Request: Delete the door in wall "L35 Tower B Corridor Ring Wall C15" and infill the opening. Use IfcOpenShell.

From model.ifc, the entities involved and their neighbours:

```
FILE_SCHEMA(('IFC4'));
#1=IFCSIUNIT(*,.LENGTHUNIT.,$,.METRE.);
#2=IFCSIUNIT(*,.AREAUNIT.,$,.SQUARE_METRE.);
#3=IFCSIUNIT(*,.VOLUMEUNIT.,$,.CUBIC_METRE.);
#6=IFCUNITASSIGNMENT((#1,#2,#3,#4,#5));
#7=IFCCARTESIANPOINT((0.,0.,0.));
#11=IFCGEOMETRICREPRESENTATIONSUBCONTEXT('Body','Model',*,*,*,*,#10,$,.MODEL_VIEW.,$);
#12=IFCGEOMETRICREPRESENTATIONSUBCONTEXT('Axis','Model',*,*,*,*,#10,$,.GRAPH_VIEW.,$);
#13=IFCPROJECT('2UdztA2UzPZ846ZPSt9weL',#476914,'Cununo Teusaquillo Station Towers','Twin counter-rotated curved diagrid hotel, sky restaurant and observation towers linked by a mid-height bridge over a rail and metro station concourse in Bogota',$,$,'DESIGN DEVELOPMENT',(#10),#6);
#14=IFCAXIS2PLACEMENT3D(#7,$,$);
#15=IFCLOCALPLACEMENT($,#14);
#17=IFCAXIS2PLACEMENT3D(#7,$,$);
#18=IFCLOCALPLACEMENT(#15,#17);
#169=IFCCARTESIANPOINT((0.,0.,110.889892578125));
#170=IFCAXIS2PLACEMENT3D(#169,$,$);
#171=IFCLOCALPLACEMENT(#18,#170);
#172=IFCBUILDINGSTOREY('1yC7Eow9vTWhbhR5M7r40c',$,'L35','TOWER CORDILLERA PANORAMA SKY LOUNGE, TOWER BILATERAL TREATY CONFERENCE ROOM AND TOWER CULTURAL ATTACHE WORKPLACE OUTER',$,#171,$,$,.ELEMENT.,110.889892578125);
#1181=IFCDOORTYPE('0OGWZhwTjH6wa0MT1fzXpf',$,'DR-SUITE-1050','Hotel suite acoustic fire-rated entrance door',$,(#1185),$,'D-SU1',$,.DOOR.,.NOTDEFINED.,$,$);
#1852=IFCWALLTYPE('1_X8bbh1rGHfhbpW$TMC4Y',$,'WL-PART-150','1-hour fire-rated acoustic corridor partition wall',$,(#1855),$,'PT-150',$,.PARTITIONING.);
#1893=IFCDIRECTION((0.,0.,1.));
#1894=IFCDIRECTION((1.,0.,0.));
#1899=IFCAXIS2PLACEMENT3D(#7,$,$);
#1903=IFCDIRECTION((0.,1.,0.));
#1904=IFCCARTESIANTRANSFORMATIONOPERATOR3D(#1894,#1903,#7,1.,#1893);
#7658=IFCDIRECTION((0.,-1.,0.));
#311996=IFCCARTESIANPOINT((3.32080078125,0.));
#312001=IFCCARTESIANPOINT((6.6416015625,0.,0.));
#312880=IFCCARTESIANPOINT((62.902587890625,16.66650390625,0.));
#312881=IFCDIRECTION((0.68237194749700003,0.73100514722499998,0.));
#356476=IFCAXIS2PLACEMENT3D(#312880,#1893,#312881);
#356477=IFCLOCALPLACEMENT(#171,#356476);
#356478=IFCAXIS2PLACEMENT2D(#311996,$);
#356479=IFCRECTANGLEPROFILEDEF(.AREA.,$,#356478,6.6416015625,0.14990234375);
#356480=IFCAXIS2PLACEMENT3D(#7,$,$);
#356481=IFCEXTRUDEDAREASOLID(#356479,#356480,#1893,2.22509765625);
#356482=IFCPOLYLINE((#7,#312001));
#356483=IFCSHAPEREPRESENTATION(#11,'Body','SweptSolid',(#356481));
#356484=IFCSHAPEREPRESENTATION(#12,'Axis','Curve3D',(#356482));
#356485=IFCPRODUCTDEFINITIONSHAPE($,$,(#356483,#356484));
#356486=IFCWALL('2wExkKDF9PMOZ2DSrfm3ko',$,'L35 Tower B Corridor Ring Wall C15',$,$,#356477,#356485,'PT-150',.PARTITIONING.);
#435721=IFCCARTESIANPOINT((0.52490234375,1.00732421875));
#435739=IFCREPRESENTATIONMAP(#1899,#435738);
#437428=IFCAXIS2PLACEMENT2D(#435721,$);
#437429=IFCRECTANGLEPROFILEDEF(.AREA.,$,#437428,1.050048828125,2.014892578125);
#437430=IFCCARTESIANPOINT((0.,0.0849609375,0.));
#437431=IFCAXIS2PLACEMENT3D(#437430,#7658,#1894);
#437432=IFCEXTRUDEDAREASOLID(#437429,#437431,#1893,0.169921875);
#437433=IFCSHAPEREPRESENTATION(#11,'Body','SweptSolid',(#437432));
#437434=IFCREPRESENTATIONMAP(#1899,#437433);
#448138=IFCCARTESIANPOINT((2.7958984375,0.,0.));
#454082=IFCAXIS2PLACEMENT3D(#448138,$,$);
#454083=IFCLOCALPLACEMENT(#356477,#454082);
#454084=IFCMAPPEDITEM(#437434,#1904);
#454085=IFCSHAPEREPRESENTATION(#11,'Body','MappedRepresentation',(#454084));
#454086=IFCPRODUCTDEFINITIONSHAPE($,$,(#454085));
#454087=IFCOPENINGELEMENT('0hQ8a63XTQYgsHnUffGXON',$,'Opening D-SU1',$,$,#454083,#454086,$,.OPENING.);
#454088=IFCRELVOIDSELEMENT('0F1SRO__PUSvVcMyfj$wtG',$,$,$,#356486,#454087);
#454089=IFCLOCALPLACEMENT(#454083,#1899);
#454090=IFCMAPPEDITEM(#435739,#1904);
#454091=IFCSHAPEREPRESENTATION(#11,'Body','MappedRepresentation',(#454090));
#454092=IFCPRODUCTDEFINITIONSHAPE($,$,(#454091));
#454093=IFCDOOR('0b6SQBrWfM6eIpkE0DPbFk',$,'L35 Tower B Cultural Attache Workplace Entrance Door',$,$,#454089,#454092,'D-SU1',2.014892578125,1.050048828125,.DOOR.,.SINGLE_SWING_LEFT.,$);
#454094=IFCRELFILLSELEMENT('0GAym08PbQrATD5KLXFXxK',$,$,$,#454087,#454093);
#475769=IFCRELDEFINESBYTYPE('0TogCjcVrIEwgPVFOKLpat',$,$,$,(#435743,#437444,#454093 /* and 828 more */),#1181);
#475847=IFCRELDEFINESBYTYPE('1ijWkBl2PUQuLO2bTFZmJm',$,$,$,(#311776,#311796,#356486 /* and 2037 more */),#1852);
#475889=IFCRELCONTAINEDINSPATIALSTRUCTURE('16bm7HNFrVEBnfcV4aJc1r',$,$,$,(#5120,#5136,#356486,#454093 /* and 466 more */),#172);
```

```python
import ifcopenshell
import ifcopenshell.api.feature
import ifcopenshell.api.root
import ifcopenshell.geom
import ifcopenshell.util.shape

model = ifcopenshell.open("model.ifc")
settings = ifcopenshell.geom.settings()


def volume(element):
    """Net volume in cubic metres, openings subtracted."""
    shape = ifcopenshell.geom.create_shape(settings, element)
    return ifcopenshell.util.shape.get_volume(shape.geometry)


door = model.by_guid("0b6SQBrWfM6eIpkE0DPbFk")
opening = door.FillsVoids[0].RelatingOpeningElement
wall = opening.VoidsElements[0].RelatingBuildingElement
before = volume(wall)

ifcopenshell.api.root.remove_product(model, product=door)
ifcopenshell.api.feature.remove_feature(model, feature=opening)

after = volume(wall)

print(f"wall volume {before:.3f} -> {after:.3f} m3")

model.write("model_rev.ifc")
```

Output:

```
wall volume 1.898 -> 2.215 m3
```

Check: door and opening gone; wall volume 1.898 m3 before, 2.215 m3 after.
